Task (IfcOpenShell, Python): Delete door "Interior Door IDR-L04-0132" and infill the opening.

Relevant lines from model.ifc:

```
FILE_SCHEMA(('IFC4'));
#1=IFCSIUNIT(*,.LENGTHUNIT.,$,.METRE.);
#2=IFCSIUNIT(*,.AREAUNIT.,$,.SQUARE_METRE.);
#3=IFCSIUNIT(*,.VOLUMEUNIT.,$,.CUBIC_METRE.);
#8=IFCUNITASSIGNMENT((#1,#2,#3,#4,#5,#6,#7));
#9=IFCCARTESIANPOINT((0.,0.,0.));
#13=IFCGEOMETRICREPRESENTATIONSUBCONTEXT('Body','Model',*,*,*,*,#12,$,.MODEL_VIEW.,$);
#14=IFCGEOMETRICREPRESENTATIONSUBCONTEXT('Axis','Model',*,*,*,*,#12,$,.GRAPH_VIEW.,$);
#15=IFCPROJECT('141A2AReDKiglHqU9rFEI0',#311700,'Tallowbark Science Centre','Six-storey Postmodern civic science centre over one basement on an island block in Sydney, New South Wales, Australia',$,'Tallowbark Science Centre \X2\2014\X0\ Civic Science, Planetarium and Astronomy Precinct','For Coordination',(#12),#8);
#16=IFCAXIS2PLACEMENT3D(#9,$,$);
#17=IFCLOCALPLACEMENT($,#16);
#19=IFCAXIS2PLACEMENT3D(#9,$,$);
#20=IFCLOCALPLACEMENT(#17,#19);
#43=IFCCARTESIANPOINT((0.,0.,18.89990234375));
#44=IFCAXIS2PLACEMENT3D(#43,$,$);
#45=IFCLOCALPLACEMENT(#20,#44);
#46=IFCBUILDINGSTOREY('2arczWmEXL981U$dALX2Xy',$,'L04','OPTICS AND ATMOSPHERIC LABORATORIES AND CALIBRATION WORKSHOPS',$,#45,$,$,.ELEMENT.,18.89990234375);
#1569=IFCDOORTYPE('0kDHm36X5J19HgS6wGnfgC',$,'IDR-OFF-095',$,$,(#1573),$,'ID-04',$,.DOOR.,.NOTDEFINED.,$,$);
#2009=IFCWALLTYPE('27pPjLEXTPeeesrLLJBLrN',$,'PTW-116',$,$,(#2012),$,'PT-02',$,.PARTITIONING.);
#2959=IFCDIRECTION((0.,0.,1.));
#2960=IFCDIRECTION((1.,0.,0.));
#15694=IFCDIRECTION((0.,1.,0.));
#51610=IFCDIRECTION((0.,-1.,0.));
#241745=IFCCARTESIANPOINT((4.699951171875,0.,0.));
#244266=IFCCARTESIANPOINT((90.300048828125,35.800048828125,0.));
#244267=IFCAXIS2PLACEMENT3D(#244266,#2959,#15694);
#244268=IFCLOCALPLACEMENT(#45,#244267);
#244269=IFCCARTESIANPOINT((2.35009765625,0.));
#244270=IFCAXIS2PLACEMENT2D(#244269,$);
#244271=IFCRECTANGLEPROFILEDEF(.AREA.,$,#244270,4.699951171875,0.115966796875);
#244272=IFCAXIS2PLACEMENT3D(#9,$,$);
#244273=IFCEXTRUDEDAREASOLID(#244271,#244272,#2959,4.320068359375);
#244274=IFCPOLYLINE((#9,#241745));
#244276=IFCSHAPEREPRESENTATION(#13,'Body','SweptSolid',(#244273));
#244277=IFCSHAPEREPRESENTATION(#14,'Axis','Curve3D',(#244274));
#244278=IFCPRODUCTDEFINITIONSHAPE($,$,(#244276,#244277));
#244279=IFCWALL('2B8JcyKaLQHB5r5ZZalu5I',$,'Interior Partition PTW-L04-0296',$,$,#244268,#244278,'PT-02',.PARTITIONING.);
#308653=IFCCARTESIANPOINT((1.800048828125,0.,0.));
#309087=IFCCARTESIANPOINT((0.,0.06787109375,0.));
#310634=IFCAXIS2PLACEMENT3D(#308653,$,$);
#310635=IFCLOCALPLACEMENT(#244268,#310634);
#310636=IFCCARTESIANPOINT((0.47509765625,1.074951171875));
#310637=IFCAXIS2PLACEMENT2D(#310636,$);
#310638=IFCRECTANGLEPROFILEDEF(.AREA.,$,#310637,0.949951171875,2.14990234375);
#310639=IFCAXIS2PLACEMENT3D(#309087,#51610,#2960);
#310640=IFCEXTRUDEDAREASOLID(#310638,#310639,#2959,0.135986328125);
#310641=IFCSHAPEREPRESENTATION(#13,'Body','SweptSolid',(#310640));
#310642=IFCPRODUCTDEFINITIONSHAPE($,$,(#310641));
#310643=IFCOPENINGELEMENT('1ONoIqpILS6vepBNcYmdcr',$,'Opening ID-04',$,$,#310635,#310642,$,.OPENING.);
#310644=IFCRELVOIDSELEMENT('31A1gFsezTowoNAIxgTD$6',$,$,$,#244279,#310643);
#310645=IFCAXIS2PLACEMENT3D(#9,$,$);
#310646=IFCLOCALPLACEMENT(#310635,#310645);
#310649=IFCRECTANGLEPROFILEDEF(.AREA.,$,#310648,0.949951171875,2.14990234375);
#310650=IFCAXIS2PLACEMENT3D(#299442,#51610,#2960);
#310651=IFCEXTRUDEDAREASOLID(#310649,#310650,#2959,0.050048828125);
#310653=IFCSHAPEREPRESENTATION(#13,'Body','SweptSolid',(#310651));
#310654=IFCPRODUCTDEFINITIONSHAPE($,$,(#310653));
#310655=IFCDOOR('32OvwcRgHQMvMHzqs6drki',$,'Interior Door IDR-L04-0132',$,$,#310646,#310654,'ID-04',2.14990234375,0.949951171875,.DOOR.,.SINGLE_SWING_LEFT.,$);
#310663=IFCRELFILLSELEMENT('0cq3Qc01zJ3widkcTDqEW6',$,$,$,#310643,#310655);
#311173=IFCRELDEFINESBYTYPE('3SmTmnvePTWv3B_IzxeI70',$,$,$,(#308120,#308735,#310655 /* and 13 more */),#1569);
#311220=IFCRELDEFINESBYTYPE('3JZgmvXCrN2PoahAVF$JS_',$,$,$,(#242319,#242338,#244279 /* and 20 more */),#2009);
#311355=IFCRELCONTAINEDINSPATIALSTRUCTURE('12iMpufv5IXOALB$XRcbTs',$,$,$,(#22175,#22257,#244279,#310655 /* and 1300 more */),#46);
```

```python
import ifcopenshell
import ifcopenshell.api.feature
import ifcopenshell.api.root
import ifcopenshell.geom
import ifcopenshell.util.shape

model = ifcopenshell.open("model.ifc")
settings = ifcopenshell.geom.settings()


def volume(element):
    """Net volume in cubic metres, openings subtracted."""
    shape = ifcopenshell.geom.create_shape(settings, element)
    return ifcopenshell.util.shape.get_volume(shape.geometry)


door = model.by_id(310655)
opening = door.FillsVoids[0].RelatingOpeningElement
wall = opening.VoidsElements[0].RelatingBuildingElement
before = volume(wall)

ifcopenshell.api.root.remove_product(model, product=door)
ifcopenshell.api.feature.remove_feature(model, feature=opening)

after = volume(wall)

print(f"wall volume {before:.3f} -> {after:.3f} m3")

model.write("model_rev.ifc")
```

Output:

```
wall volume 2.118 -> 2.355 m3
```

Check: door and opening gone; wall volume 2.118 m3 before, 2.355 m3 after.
